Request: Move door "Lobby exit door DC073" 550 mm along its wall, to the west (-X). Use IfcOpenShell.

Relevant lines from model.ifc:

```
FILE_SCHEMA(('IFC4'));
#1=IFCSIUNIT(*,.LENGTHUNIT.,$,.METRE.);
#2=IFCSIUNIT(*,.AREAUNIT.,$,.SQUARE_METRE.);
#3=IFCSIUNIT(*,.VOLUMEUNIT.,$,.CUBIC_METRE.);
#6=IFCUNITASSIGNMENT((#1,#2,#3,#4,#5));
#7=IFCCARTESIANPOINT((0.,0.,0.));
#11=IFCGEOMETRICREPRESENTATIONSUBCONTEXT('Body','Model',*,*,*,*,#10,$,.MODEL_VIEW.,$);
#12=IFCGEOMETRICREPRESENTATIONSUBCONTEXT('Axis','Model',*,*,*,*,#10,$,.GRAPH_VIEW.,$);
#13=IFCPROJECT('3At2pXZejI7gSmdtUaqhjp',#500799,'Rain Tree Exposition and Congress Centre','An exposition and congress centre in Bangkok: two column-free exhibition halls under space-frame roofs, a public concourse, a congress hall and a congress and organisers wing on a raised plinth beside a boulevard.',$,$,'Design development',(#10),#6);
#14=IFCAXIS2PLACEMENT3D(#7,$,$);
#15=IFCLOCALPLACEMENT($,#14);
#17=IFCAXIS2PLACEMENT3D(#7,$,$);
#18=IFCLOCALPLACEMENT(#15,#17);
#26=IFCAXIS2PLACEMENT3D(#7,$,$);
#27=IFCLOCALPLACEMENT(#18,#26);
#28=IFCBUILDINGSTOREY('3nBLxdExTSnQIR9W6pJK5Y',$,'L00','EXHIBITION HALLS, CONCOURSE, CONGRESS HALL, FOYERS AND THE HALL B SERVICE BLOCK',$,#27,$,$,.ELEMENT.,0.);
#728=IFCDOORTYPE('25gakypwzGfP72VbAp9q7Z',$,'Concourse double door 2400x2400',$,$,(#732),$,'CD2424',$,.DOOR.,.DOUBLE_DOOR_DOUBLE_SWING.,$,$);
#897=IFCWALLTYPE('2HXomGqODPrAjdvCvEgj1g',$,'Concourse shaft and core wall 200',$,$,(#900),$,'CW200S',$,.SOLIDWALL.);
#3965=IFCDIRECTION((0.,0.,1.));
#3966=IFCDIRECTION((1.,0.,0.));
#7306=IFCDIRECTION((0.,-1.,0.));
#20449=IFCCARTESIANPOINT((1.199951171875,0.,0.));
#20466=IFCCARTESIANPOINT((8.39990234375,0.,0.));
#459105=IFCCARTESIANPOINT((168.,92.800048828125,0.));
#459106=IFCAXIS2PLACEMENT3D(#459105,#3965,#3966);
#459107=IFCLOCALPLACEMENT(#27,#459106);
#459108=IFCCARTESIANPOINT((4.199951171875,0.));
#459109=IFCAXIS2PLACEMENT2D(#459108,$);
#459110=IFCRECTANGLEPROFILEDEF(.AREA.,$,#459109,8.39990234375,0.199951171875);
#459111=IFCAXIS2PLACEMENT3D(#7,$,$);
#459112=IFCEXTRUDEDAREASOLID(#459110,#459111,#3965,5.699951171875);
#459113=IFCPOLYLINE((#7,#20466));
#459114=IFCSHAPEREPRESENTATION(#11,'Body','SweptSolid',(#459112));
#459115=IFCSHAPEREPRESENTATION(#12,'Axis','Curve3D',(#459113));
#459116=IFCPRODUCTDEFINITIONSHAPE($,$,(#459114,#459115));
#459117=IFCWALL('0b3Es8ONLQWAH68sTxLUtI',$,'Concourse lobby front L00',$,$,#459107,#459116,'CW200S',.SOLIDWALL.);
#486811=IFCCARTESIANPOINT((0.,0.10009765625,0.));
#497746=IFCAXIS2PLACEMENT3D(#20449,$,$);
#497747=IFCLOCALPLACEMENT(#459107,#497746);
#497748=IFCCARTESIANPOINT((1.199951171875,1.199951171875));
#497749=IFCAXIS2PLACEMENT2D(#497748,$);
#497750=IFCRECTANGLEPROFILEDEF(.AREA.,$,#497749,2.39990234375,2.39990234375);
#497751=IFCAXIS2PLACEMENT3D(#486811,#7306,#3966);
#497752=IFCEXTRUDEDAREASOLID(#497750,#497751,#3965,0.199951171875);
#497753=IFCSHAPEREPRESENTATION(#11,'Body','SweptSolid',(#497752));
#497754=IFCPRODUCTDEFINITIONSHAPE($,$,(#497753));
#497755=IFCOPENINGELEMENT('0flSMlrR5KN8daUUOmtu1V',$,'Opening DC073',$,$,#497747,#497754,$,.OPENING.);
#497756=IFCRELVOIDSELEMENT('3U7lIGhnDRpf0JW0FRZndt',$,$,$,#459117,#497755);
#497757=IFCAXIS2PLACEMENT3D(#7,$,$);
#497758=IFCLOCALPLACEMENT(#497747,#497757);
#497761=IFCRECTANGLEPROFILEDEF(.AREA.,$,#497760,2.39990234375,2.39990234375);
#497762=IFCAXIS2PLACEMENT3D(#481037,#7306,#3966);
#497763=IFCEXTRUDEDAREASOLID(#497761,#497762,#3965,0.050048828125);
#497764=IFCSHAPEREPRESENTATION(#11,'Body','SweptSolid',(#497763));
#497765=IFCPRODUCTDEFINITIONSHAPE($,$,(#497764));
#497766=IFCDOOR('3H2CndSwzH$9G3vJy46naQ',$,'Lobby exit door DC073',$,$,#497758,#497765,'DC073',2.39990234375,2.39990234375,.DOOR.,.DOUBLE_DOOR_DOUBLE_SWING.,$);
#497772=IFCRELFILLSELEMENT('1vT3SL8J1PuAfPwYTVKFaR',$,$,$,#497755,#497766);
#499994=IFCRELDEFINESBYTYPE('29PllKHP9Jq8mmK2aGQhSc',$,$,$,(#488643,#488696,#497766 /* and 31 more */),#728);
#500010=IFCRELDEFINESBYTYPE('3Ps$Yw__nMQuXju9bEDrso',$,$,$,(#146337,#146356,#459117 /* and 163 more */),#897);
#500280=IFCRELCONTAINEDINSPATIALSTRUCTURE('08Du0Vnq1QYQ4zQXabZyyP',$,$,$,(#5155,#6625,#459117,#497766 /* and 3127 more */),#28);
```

```python
import ifcopenshell
import ifcopenshell.api.geometry
import ifcopenshell.util.placement
import ifcopenshell.util.unit

model = ifcopenshell.open("model.ifc")
unit_scale = ifcopenshell.util.unit.calculate_unit_scale(model)

door = model.by_guid("3H2CndSwzH$9G3vJy46naQ")
opening = door.FillsVoids[0].RelatingOpeningElement
wall = opening.VoidsElements[0].RelatingBuildingElement

wall_matrix = ifcopenshell.util.placement.get_local_placement(wall.ObjectPlacement)
shift = wall_matrix[:3, 0] * -0.55 / unit_scale
before = ifcopenshell.util.placement.get_local_placement(door.ObjectPlacement)[:3, 3].copy()

# The door is placed relative to its opening, so it follows when the opening moves.
matrix = ifcopenshell.util.placement.get_local_placement(opening.ObjectPlacement)
matrix[:3, 3] += shift
ifcopenshell.api.geometry.edit_object_placement(
    model, product=opening, matrix=matrix, is_si=False, should_transform_children=True
)

after = ifcopenshell.util.placement.get_local_placement(door.ObjectPlacement)[:3, 3]
print("door moved by", (after - before).round(3) + 0.0)

model.write("model-out.ifc")
```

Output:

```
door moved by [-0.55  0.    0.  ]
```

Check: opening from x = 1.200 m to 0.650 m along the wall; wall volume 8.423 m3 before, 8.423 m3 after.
